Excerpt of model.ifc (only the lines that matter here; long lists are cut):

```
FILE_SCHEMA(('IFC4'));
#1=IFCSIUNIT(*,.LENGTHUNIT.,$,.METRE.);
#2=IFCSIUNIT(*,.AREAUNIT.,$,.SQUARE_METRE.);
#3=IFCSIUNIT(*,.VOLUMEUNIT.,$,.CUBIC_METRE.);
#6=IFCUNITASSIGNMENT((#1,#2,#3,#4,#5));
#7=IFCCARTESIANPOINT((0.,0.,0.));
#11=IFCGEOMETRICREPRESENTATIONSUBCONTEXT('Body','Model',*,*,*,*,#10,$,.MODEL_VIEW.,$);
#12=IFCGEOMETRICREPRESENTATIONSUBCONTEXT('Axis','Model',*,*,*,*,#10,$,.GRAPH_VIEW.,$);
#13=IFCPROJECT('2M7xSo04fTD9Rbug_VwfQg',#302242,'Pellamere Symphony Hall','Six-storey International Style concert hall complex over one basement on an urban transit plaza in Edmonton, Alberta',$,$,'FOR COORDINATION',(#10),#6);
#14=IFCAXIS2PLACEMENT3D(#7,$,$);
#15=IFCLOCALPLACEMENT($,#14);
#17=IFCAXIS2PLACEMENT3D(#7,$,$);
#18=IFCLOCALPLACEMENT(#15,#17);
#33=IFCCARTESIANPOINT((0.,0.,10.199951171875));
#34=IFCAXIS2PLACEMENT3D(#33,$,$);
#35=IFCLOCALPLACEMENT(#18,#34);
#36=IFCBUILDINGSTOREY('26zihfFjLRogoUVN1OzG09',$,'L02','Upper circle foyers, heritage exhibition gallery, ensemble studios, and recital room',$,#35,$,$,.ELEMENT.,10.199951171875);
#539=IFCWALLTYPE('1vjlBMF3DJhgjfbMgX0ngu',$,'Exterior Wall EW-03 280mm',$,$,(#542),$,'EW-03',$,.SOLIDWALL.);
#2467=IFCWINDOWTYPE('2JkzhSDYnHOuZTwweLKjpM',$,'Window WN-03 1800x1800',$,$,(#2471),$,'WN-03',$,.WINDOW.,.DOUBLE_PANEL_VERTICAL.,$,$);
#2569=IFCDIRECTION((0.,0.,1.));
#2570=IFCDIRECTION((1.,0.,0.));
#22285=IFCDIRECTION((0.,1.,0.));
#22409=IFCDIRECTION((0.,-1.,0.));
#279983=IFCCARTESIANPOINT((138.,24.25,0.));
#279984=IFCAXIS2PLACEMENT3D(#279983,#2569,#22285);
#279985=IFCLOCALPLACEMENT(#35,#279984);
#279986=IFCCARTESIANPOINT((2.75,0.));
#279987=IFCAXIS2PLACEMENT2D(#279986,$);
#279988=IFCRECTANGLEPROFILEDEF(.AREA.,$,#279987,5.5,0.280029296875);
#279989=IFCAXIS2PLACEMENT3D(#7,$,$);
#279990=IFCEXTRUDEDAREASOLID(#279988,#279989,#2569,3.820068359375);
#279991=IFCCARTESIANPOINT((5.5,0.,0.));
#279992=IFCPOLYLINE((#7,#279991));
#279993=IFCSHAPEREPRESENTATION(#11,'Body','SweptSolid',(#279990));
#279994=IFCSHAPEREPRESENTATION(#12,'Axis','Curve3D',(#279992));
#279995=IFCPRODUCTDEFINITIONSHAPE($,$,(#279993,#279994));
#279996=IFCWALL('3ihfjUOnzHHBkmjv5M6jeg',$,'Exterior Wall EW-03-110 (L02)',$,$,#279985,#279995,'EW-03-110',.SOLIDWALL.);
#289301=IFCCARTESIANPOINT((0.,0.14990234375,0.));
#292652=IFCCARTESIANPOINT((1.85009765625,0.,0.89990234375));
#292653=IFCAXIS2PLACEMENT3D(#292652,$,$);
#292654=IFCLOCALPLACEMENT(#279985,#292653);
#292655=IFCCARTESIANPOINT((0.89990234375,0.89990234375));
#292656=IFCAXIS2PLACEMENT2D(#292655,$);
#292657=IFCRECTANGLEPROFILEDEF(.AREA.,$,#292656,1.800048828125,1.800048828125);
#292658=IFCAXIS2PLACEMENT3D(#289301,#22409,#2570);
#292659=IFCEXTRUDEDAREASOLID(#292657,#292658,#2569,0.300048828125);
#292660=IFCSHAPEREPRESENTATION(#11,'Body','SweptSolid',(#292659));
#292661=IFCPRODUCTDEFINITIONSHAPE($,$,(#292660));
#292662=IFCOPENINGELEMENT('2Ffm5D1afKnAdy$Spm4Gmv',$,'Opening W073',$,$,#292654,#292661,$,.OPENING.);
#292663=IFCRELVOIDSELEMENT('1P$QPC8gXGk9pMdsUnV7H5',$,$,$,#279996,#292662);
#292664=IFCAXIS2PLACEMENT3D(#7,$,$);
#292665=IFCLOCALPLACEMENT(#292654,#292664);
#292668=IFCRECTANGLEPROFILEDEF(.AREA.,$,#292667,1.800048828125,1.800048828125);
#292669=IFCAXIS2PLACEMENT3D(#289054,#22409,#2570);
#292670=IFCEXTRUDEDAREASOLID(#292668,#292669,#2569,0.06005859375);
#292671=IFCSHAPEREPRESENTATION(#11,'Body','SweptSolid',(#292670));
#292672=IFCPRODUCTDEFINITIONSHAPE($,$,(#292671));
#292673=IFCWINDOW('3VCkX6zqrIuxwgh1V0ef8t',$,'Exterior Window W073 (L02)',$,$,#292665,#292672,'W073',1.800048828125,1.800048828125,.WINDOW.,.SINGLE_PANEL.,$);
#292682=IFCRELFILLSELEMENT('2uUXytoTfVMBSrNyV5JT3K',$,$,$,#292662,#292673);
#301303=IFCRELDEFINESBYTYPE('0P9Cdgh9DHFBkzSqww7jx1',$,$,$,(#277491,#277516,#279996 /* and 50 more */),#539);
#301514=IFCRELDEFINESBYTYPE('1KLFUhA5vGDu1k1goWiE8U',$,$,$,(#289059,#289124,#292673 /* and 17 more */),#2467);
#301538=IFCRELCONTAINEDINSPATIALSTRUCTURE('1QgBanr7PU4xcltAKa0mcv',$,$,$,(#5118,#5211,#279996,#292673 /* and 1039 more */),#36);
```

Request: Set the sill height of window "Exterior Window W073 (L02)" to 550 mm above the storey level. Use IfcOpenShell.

```python
import numpy as np
import ifcopenshell
import ifcopenshell.api.geometry
import ifcopenshell.geom
import ifcopenshell.util.element
import ifcopenshell.util.placement
import ifcopenshell.util.shape
import ifcopenshell.util.unit

model = ifcopenshell.open("model.ifc")
unit_scale = ifcopenshell.util.unit.calculate_unit_scale(model)

window = model.by_guid("3VCkX6zqrIuxwgh1V0ef8t")
opening = window.FillsVoids[0].RelatingOpeningElement
storey = ifcopenshell.util.element.get_container(window, ifc_class="IfcBuildingStorey")
level = ifcopenshell.util.placement.get_local_placement(storey.ObjectPlacement)[2, 3]

# The opening's origin need not be at the sill, so measure its lowest point.
shape = ifcopenshell.geom.create_shape(ifcopenshell.geom.settings(), opening)
bottom = ifcopenshell.util.shape.get_shape_bottom_elevation(shape, shape.geometry) / unit_scale
dz = level + 0.55 / unit_scale - bottom

shift = np.array([0.0, 0.0, dz])
# The window is placed relative to its opening, so it follows when the opening moves.
matrix = ifcopenshell.util.placement.get_local_placement(opening.ObjectPlacement)
matrix[:3, 3] += shift
ifcopenshell.api.geometry.edit_object_placement(
    model, product=opening, matrix=matrix, is_si=False, should_transform_children=True
)

print(f"moved by {dz * unit_scale:+.3f} m")

model.write("model_edited.ifc")
```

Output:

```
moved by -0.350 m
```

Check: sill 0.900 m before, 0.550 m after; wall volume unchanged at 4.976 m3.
